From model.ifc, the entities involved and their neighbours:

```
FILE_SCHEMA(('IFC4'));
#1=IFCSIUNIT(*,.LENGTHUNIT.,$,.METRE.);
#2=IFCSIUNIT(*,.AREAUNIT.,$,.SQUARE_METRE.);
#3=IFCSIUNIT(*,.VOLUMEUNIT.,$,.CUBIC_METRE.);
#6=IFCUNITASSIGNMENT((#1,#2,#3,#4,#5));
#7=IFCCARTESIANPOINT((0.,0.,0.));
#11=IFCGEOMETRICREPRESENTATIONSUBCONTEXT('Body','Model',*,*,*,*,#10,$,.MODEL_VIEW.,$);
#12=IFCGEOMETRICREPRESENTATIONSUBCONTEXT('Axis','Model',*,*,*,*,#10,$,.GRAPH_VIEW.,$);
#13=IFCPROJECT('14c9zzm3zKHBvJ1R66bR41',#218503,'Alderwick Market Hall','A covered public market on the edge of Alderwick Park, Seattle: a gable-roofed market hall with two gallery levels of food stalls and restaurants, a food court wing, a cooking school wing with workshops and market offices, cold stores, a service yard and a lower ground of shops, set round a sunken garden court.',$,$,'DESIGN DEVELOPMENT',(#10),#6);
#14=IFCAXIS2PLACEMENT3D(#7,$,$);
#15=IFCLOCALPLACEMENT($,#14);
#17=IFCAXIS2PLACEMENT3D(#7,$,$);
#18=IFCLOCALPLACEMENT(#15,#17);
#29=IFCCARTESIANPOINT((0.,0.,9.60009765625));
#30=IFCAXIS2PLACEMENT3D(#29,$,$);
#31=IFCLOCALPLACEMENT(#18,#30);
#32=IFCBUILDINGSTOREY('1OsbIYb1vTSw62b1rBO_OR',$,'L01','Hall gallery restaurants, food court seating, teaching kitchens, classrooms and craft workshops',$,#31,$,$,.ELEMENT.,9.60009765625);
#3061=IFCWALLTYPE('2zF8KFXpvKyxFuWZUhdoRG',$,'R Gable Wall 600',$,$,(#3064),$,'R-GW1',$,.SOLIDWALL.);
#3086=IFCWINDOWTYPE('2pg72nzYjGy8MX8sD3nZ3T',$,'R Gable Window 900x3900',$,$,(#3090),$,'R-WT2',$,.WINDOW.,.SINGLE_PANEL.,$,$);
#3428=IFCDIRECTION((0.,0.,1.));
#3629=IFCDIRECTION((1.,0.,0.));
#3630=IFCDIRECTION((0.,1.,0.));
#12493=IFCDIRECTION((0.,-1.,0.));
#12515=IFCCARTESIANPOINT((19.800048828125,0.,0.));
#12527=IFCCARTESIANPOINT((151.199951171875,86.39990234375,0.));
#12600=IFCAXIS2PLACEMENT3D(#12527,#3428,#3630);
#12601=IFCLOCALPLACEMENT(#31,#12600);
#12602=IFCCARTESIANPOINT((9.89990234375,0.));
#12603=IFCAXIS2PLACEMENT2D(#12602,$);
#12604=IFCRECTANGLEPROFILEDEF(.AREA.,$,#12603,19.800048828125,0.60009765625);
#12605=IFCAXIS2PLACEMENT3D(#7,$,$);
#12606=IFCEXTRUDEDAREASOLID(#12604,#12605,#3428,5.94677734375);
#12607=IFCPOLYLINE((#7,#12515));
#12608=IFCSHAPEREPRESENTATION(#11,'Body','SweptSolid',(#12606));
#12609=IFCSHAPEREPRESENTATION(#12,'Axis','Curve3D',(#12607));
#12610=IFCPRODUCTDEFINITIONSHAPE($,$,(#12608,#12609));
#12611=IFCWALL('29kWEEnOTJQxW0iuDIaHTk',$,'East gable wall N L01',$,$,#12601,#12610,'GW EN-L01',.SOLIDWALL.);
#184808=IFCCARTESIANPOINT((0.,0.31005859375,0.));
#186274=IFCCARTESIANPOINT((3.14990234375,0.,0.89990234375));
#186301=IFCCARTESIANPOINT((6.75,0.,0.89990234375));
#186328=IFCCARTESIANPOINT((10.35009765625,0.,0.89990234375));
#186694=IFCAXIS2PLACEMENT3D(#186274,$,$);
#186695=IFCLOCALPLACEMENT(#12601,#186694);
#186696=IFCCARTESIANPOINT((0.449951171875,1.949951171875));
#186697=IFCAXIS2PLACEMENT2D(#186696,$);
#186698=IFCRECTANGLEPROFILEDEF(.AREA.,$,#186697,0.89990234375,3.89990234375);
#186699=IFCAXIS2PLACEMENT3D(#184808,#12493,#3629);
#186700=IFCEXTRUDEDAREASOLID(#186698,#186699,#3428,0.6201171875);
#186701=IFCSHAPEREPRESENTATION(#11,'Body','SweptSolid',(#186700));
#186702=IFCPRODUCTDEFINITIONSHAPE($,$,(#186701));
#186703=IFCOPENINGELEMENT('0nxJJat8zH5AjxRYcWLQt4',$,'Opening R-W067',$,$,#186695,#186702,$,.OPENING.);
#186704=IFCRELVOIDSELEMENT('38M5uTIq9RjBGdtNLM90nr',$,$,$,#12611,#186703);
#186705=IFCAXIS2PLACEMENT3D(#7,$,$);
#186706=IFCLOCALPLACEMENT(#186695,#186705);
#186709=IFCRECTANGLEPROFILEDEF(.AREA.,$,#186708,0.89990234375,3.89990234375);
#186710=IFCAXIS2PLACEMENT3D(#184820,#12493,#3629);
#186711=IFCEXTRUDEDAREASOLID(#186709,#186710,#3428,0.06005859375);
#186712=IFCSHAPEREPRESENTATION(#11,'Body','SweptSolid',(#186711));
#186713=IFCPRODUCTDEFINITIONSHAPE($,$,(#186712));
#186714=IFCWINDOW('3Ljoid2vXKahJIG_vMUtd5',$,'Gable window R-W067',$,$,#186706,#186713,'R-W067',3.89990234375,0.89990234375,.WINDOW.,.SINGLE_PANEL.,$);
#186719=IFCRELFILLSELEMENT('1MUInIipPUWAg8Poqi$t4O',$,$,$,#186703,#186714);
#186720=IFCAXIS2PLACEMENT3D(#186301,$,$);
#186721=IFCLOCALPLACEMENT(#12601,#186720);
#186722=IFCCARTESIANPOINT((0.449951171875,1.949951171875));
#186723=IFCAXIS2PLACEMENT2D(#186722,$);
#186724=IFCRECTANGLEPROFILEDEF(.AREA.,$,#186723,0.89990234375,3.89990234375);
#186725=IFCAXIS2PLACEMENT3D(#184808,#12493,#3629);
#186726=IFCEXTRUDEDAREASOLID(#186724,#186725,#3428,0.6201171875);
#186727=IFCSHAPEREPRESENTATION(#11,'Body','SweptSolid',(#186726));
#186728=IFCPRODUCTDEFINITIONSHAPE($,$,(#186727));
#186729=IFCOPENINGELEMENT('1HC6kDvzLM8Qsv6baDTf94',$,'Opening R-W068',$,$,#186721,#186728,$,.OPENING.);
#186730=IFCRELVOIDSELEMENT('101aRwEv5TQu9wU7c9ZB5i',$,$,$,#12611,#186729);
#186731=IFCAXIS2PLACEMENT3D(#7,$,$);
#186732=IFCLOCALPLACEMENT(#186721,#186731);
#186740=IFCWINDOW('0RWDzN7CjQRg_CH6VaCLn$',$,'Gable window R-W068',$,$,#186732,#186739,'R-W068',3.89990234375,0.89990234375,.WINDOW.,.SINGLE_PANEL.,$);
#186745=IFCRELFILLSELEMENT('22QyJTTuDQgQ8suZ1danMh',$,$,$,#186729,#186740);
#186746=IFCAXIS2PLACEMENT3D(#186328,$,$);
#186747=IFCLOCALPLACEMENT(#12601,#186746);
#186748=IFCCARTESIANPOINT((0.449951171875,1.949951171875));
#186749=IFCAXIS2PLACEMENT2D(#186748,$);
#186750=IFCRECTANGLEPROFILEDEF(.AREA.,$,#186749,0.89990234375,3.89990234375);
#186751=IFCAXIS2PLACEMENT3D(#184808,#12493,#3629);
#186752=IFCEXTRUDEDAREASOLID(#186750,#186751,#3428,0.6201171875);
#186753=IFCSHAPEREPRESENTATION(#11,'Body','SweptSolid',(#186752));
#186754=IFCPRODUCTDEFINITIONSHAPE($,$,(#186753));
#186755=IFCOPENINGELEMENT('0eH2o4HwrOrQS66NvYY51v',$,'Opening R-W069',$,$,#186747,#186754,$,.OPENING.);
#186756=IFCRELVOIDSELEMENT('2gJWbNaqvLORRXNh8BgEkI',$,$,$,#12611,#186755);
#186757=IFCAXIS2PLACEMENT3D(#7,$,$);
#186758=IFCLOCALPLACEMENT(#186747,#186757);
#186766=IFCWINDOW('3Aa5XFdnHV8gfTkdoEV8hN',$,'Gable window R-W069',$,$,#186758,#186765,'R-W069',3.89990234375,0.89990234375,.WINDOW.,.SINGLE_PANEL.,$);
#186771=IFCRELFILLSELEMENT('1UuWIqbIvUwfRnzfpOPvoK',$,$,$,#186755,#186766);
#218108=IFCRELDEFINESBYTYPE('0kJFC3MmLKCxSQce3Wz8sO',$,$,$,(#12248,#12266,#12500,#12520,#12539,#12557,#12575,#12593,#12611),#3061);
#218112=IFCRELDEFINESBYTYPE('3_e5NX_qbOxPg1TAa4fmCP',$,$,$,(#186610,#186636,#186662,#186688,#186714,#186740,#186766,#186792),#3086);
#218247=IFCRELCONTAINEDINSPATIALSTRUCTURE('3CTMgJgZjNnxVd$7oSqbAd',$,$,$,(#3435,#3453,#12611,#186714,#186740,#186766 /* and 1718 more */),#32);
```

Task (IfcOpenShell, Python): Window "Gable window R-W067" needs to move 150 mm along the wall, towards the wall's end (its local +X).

```python
import ifcopenshell
import ifcopenshell.api.geometry
import ifcopenshell.util.placement

model = ifcopenshell.open("model.ifc")

window = model.by_id(186714)
opening = window.FillsVoids[0].RelatingOpeningElement
wall = opening.VoidsElements[0].RelatingBuildingElement

wall_matrix = ifcopenshell.util.placement.get_local_placement(wall.ObjectPlacement)
shift = wall_matrix[:3, 0] * 0.15
before = ifcopenshell.util.placement.get_local_placement(window.ObjectPlacement)[:3, 3].copy()

# The window is placed relative to its opening, so it follows when the opening moves.
matrix = ifcopenshell.util.placement.get_local_placement(opening.ObjectPlacement)
matrix[:3, 3] += shift
ifcopenshell.api.geometry.edit_object_placement(
    model, product=opening, matrix=matrix, is_si=False, should_transform_children=True
)

after = ifcopenshell.util.placement.get_local_placement(window.ObjectPlacement)[:3, 3]
print("window moved by", (after - before).round(3) + 0.0)

model.write("model_rev.ifc")
```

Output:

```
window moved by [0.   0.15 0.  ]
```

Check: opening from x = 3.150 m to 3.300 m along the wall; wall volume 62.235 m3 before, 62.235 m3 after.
